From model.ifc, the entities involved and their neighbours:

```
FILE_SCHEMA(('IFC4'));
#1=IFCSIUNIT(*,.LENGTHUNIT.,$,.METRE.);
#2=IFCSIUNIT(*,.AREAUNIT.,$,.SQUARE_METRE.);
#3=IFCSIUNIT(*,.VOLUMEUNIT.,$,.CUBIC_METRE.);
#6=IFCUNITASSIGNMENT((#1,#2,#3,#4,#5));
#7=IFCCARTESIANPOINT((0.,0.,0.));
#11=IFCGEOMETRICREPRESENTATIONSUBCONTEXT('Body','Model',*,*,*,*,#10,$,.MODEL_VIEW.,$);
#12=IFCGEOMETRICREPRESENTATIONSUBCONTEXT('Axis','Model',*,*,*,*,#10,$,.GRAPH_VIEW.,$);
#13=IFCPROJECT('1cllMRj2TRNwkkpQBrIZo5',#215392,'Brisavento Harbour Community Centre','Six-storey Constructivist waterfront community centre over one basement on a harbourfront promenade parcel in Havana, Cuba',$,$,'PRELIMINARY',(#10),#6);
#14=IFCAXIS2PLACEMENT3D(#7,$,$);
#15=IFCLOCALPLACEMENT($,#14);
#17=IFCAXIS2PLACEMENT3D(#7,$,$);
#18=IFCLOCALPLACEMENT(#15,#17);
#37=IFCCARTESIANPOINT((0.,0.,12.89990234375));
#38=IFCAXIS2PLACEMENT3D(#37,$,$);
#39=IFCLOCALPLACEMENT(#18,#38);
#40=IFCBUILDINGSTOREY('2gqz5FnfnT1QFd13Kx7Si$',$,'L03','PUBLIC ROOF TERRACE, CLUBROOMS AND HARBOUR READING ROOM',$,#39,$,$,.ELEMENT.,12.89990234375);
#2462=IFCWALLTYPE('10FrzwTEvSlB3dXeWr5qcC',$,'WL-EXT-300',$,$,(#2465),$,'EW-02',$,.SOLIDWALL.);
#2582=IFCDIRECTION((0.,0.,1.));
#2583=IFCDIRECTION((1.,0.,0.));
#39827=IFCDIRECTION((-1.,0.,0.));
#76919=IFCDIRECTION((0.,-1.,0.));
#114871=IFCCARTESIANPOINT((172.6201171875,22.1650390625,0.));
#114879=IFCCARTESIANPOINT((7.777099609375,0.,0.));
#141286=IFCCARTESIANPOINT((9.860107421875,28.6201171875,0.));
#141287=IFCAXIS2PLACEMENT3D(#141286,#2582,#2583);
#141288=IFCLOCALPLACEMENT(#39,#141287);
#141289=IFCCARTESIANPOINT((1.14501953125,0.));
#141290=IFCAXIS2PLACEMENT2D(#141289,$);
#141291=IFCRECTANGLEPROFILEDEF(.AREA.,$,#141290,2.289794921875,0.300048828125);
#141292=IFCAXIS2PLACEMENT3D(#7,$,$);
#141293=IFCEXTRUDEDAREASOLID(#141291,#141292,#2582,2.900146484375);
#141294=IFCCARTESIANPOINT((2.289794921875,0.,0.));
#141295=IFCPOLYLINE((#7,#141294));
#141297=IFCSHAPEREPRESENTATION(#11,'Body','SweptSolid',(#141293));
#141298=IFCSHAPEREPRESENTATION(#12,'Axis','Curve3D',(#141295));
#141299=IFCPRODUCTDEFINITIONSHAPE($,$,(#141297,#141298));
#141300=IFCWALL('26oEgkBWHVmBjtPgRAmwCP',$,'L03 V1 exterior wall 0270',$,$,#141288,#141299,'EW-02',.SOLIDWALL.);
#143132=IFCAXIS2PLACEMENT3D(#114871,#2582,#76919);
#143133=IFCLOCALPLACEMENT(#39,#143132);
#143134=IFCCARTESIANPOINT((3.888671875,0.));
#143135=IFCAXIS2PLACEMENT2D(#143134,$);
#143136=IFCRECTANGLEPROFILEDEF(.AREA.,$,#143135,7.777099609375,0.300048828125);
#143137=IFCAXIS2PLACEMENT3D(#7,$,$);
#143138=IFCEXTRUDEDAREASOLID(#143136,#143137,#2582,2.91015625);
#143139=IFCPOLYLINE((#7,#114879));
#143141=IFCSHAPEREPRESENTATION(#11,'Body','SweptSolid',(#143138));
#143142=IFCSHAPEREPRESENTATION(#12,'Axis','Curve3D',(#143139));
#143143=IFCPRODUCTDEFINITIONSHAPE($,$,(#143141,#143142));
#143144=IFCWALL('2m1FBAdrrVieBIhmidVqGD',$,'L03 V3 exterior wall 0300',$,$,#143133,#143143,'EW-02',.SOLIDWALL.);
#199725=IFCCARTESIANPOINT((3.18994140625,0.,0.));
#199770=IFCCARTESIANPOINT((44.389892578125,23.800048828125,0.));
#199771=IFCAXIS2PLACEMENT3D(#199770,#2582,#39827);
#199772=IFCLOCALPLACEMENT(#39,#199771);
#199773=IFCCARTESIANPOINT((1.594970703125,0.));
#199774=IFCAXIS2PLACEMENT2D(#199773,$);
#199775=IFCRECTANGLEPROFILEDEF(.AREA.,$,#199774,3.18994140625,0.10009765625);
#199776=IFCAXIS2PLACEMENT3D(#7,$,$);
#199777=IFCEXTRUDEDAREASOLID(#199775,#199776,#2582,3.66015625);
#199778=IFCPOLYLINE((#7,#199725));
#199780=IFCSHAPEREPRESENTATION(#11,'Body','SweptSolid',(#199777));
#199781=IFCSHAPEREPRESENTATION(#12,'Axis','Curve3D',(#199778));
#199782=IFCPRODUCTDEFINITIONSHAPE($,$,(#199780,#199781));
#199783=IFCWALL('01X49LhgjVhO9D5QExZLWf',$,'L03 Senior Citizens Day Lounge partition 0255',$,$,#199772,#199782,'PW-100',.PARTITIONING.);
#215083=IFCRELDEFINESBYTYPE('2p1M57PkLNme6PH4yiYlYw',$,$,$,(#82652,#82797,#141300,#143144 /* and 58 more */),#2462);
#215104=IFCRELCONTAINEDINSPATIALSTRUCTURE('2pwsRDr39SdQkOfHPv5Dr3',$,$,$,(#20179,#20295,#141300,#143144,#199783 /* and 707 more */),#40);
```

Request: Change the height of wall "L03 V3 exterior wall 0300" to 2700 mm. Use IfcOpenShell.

```python
import ifcopenshell
import ifcopenshell.geom
import ifcopenshell.util.representation
import ifcopenshell.util.shape
import ifcopenshell.util.unit

model = ifcopenshell.open("model.ifc")
unit_scale = ifcopenshell.util.unit.calculate_unit_scale(model)
settings = ifcopenshell.geom.settings()


def volume(element):
    """Net volume in cubic metres, openings subtracted."""
    shape = ifcopenshell.geom.create_shape(settings, element)
    return ifcopenshell.util.shape.get_volume(shape.geometry)


wall = model.by_guid("2m1FBAdrrVieBIhmidVqGD")
before = volume(wall)

body = ifcopenshell.util.representation.get_representation(wall, "Model", "Body")
solid = body.Items[0]
old_height = solid.Depth
solid.Depth = 2.7 / unit_scale
after = volume(wall)

print(f"height {old_height:g} -> {solid.Depth:g}, volume {before:.3f} -> {after:.3f} m3")

model.write("model_v2.ifc")
```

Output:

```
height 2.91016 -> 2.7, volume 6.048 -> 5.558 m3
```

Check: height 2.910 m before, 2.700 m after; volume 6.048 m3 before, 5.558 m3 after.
